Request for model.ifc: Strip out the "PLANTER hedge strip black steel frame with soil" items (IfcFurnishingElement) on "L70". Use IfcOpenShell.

First a look at what the model holds.

```python
import ifcopenshell
import ifcopenshell.util.element

model = ifcopenshell.open("model.ifc")
print(model.schema)
storey = next(s for s in model.by_type("IfcBuildingStorey") if s.Name == "L70")
furniture = [e for e in ifcopenshell.util.element.get_decomposition(storey) if e.is_a("IfcFurnishingElement")]
seen = {}
for e in furniture:
    element_type = ifcopenshell.util.element.get_type(e)
    name = element_type.Name if element_type not in (None, e) else None
    seen[name] = seen.get(name, 0) + 1
for name, count in sorted(seen.items(), key=str):
    print(count, "x", name)
```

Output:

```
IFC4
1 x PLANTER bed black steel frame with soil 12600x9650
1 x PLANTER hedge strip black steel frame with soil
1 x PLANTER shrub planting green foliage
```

```python
import ifcopenshell
import ifcopenshell.api.root
import ifcopenshell.util.element

model = ifcopenshell.open("model.ifc")

storey = next(s for s in model.by_type("IfcBuildingStorey") if s.Name == "L70")
furniture = [e for e in ifcopenshell.util.element.get_decomposition(storey) if e.is_a("IfcFurnishingElement")]
targets = [e for e in furniture if (t := ifcopenshell.util.element.get_type(e)) not in (None, e) and t.Name == "PLANTER hedge strip black steel frame with soil"]

for e in targets:
    ifcopenshell.api.root.remove_product(model, product=e)
print(len(targets), "removed")

model.write("model_edited.ifc")
```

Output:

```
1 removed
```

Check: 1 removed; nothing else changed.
